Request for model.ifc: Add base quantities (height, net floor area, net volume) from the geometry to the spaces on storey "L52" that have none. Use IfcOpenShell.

First a look at what the model holds.

```python
import ifcopenshell
import ifcopenshell.util.element
import ifcopenshell.util.unit

model = ifcopenshell.open("model.ifc")
print(model.schema)
for unit_type in ("LENGTHUNIT", "AREAUNIT", "VOLUMEUNIT"):
    print(unit_type, ifcopenshell.util.unit.calculate_unit_scale(model, unit_type))
storey = next(s for s in model.by_type("IfcBuildingStorey") if s.Name == "L52")
spaces = [e for e in ifcopenshell.util.element.get_decomposition(storey) if e.is_a("IfcSpace")]
for e in sorted(spaces, key=lambda e: e.id()):
    print(e.id(), e.is_a(), e.Name, list(ifcopenshell.util.element.get_psets(e, qtos_only=True)), sep=" | ")
```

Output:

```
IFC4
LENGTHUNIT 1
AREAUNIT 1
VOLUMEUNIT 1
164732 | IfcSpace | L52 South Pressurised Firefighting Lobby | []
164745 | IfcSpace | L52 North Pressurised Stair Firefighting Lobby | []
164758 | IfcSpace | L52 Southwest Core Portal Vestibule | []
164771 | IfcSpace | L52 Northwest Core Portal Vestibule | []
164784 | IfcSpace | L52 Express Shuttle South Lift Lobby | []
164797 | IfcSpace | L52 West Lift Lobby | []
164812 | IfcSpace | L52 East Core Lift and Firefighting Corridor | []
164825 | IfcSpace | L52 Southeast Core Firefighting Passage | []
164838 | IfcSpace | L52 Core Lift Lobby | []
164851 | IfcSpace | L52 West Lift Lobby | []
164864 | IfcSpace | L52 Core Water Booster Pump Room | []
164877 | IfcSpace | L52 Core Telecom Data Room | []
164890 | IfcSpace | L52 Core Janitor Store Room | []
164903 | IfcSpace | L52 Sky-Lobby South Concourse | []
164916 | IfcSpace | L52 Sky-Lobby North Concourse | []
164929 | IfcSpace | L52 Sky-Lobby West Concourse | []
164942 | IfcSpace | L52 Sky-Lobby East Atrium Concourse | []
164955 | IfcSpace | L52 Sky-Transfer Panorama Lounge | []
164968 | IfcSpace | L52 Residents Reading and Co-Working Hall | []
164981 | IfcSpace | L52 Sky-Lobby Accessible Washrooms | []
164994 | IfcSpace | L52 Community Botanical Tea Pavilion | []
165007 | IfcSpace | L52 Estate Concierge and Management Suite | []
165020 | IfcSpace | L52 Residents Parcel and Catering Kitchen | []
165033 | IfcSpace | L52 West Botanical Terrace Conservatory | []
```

```python
import ifcopenshell
import ifcopenshell.api.pset
import ifcopenshell.geom
import ifcopenshell.util.element
import ifcopenshell.util.shape
import ifcopenshell.util.unit

model = ifcopenshell.open("model.ifc")
unit_scale = ifcopenshell.util.unit.calculate_unit_scale(model)
area_scale = ifcopenshell.util.unit.calculate_unit_scale(model, "AREAUNIT")
volume_scale = ifcopenshell.util.unit.calculate_unit_scale(model, "VOLUMEUNIT")
settings = ifcopenshell.geom.settings()

storey = next(s for s in model.by_type("IfcBuildingStorey") if s.Name == "L52")
spaces = [e for e in ifcopenshell.util.element.get_decomposition(storey) if e.is_a("IfcSpace")]

for e in sorted(spaces, key=lambda e: e.id()):
    if ifcopenshell.util.element.get_psets(e, qtos_only=True, should_inherit=False):
        continue
    # Geometry comes back in metres, in the element's own axes.
    shape = ifcopenshell.geom.create_shape(settings, e)
    values = {
        "Height": ifcopenshell.util.shape.get_z(shape.geometry) / unit_scale,
        "NetFloorArea": ifcopenshell.util.shape.get_footprint_area(shape.geometry) / area_scale,
        "NetVolume": ifcopenshell.util.shape.get_volume(shape.geometry) / volume_scale,
    }
    qto = ifcopenshell.api.pset.add_qto(model, product=e, name="Qto_SpaceBaseQuantities")
    ifcopenshell.api.pset.edit_qto(model, qto=qto, properties=values)
    print(e.id(), {k: round(v, 3) for k, v in values.items()})

model.write("model-out.ifc")
```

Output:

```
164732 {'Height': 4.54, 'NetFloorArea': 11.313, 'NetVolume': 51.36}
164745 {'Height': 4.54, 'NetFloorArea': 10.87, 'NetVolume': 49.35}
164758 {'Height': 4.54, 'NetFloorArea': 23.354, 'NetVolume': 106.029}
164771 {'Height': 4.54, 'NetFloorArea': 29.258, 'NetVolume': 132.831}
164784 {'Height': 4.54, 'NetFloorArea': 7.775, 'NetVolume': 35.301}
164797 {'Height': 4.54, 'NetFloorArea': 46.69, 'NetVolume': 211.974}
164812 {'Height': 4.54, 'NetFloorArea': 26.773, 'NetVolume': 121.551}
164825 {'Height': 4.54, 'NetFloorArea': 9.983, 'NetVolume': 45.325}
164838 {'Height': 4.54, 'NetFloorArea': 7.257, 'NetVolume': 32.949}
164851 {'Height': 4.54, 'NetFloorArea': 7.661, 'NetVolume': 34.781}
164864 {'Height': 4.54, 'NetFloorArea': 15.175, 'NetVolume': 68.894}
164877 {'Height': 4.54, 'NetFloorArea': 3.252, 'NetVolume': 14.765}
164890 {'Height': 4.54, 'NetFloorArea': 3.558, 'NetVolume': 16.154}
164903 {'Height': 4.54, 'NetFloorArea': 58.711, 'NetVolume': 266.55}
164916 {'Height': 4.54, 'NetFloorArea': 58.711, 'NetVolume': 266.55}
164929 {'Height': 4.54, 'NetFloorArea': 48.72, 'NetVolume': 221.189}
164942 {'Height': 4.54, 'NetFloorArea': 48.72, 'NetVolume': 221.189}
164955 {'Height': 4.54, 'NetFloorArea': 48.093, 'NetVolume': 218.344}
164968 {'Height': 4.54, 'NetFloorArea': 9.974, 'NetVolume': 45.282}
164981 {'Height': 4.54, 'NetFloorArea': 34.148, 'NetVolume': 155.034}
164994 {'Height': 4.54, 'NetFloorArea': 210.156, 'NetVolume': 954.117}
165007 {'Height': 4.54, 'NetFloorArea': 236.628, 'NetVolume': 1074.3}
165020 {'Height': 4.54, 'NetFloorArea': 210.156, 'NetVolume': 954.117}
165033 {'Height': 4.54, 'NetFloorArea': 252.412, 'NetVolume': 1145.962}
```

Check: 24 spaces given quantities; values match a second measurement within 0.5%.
